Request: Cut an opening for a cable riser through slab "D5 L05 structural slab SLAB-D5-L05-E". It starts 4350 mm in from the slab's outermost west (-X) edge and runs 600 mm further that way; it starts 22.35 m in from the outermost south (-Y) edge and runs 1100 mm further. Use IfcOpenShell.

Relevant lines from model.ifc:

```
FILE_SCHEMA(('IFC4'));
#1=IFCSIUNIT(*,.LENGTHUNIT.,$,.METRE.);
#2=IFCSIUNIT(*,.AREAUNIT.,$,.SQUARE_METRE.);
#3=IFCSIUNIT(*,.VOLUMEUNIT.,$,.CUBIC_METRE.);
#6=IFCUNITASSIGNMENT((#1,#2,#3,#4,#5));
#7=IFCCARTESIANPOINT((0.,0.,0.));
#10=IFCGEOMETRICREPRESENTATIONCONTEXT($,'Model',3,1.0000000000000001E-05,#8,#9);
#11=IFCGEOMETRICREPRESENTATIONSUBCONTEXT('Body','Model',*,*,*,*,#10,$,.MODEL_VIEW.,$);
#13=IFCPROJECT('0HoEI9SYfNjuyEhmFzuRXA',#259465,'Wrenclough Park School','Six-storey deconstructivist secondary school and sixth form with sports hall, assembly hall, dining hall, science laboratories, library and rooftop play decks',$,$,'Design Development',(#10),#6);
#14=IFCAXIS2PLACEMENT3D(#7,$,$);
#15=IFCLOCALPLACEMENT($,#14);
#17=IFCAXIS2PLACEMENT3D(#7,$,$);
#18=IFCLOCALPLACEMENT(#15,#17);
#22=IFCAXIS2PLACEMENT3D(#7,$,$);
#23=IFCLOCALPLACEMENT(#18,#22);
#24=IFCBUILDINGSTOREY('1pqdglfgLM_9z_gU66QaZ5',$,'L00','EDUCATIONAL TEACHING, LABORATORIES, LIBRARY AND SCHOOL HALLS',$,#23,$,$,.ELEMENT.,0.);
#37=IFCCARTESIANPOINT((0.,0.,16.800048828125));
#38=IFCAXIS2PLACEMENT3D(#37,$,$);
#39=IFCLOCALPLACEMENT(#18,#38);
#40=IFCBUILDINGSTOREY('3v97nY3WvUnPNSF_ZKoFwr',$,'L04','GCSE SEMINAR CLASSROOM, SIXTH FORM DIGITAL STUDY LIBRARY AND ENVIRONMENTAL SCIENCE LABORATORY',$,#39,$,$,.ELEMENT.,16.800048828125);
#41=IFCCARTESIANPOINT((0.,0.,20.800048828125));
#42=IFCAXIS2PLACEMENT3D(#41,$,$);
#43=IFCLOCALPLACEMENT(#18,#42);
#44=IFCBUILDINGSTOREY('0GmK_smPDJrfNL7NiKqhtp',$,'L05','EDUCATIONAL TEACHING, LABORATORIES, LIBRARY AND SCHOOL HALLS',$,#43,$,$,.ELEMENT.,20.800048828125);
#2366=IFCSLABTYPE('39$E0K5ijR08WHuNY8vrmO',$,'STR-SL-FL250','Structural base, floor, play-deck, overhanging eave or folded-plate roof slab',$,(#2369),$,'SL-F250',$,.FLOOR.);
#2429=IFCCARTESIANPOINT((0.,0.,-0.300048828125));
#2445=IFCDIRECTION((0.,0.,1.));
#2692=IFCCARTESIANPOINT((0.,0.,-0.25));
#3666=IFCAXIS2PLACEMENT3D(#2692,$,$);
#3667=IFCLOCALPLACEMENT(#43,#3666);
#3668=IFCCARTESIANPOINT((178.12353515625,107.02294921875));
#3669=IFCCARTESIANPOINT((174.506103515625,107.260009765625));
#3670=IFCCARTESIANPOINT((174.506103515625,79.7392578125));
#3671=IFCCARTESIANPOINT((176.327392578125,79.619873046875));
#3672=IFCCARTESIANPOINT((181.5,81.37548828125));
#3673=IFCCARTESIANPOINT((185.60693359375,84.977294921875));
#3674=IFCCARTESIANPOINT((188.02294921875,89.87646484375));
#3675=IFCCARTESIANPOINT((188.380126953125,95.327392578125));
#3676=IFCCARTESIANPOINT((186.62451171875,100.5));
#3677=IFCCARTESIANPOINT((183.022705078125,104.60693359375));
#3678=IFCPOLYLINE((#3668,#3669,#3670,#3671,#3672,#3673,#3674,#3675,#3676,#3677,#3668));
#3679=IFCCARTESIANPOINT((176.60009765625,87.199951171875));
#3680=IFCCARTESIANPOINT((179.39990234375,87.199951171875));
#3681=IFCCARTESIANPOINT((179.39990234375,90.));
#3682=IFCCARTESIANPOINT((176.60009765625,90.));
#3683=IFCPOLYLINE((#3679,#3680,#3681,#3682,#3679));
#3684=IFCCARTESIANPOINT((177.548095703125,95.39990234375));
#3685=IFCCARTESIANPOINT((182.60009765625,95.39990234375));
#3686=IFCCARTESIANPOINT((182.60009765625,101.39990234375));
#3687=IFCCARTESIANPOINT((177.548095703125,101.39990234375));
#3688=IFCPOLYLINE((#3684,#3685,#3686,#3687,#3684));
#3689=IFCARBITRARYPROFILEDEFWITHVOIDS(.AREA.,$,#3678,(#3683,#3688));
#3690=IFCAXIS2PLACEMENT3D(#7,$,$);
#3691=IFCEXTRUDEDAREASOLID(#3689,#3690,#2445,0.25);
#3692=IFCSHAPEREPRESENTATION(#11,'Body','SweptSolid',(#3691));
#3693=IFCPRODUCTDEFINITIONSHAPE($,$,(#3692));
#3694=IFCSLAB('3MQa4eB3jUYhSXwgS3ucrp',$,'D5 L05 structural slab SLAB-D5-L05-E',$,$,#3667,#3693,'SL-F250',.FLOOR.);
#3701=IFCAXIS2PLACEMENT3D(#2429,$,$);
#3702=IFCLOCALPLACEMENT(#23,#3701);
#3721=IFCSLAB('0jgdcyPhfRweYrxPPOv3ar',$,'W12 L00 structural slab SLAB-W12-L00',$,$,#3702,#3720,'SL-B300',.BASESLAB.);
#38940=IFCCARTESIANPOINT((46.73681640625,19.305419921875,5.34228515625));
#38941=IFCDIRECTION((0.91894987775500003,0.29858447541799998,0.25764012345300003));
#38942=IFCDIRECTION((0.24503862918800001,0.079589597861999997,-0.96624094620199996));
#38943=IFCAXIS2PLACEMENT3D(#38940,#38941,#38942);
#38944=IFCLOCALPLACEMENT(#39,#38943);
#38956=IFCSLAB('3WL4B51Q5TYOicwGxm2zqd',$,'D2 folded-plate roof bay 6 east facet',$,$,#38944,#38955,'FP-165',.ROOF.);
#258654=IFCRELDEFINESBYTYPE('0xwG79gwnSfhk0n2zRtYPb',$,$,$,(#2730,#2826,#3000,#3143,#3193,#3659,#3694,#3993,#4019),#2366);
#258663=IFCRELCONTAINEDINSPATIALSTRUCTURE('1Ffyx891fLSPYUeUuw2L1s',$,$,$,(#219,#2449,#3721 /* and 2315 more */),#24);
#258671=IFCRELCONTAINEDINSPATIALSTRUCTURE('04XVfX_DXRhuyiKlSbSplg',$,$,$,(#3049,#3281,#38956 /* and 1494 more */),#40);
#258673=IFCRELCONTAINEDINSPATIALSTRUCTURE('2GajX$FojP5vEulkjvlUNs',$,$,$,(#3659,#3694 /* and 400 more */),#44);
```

```python
import numpy as np
import ifcopenshell
import ifcopenshell.api.feature
import ifcopenshell.api.geometry
import ifcopenshell.api.root
import ifcopenshell.geom
import ifcopenshell.util.placement
import ifcopenshell.util.representation
import ifcopenshell.util.shape
import ifcopenshell.util.unit

model = ifcopenshell.open("model.ifc")
unit_scale = ifcopenshell.util.unit.calculate_unit_scale(model)
settings = ifcopenshell.geom.settings()


def volume(element):
    """Net volume in cubic metres, openings subtracted."""
    shape = ifcopenshell.geom.create_shape(settings, element)
    return ifcopenshell.util.shape.get_volume(shape.geometry)


slab = model.by_id(3694)
before = volume(slab)

# Extent in the slab's own axes, in metres. The edges named are its -X and -Y sides.
slab_shape = ifcopenshell.geom.create_shape(settings, slab)
vertices = ifcopenshell.util.shape.get_vertices(slab_shape.geometry)
x_min, y_min, bottom = vertices.min(axis=0)
top = vertices[:, 2].max()

opening = ifcopenshell.api.root.create_entity(model, ifc_class="IfcOpeningElement", name="Cable riser opening", predefined_type="OPENING")
context = ifcopenshell.util.representation.get_context(model, "Model", "Body", "MODEL_VIEW")
width, depth = 0.6, 1.1
outline = [(0.0, 0.0), (width, 0.0), (width, depth), (0.0, depth), (0.0, 0.0)]
# Overshoot both faces by 50 mm so the cut is clean.
shape = ifcopenshell.api.geometry.add_slab_representation(
    model, context=context, depth=top - bottom + 0.1, polyline=outline
)
ifcopenshell.api.geometry.assign_representation(model, product=opening, representation=shape)

matrix = ifcopenshell.util.placement.get_local_placement(slab.ObjectPlacement)
matrix[:, 3] = matrix @ np.append(np.array([x_min + 4.35, y_min + 22.35, bottom - 0.05]) / unit_scale, 1.0)
ifcopenshell.api.geometry.edit_object_placement(model, product=opening, matrix=matrix, is_si=False)
ifcopenshell.api.feature.add_feature(model, feature=opening, element=slab)

after = volume(slab)

print(f"slab volume {before:.3f} -> {after:.3f} m3")

model.write("model-out.ifc")
```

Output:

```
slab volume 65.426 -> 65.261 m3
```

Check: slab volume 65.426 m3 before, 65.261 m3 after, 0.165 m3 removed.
